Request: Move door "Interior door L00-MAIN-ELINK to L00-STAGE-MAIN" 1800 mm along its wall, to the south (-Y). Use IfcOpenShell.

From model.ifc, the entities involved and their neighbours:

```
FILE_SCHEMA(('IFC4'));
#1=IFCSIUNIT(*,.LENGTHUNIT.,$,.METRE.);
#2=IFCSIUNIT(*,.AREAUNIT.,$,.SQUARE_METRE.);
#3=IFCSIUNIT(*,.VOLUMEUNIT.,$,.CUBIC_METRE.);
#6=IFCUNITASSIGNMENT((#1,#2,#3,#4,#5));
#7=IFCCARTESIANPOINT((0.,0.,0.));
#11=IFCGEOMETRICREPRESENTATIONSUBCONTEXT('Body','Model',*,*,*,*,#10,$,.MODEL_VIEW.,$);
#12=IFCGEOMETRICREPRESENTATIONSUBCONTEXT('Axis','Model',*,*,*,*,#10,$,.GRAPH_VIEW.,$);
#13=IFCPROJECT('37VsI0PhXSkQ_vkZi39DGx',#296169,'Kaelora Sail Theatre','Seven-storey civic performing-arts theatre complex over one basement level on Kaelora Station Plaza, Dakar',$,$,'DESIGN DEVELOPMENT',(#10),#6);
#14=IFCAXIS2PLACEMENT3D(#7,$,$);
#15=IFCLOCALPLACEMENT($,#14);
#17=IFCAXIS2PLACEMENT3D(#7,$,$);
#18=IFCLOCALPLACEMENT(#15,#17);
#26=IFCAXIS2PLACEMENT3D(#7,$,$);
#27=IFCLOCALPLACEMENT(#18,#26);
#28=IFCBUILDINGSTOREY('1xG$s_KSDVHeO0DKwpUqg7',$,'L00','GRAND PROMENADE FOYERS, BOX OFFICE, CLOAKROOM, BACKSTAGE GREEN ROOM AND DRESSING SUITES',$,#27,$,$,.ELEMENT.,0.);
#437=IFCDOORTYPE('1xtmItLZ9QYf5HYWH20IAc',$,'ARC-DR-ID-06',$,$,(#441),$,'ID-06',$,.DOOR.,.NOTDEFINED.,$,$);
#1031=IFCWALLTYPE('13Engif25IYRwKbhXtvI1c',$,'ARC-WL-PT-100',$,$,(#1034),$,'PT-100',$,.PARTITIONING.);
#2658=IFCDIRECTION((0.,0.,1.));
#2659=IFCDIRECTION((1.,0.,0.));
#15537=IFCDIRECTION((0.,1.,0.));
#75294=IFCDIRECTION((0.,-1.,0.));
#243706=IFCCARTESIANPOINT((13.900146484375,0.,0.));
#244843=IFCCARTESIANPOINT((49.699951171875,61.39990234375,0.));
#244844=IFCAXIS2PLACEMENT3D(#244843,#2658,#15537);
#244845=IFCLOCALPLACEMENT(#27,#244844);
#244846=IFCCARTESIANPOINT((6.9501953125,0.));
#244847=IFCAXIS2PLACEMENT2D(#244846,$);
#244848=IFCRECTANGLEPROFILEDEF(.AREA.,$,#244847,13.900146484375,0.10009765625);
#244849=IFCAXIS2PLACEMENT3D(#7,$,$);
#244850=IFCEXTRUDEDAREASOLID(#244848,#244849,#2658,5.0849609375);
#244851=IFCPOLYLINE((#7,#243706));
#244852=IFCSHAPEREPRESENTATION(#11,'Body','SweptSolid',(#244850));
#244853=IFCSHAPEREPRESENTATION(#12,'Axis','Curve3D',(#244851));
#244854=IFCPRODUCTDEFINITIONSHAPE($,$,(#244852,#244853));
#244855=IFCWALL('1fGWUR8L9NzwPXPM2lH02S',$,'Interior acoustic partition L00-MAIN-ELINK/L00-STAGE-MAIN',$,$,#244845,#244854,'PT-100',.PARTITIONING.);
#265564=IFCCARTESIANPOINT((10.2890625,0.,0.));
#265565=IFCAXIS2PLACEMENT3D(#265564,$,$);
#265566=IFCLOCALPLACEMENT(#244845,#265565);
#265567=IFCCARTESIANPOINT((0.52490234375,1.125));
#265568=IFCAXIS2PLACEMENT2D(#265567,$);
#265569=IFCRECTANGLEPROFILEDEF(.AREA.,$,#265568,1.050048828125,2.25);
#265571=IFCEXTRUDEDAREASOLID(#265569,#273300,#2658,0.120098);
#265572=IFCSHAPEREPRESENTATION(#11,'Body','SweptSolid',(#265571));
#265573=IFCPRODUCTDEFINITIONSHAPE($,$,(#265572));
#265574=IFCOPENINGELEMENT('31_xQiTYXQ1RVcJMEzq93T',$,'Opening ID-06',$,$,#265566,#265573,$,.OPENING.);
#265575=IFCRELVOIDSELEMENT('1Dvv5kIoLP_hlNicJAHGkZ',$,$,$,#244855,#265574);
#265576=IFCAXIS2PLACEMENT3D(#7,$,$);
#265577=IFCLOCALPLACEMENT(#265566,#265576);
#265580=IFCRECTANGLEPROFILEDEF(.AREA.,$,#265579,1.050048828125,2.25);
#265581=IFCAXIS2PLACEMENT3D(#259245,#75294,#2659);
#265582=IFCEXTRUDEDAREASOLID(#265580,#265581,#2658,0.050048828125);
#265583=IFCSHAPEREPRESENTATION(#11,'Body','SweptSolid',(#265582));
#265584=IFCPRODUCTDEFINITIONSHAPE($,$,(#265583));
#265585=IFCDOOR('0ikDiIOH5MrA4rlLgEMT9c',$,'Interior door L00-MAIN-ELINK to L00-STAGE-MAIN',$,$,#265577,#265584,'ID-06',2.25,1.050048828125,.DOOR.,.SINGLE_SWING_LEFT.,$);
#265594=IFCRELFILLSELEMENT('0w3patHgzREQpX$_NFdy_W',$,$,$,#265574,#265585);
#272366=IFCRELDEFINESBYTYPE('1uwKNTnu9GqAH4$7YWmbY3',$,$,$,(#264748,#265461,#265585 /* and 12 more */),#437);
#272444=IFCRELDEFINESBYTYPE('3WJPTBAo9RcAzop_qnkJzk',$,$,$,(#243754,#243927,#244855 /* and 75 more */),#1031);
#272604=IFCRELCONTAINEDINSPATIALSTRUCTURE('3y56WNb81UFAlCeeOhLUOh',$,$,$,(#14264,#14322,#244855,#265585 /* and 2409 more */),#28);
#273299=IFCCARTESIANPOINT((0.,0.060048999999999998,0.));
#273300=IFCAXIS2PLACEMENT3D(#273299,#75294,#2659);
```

```python
import ifcopenshell
import ifcopenshell.api.geometry
import ifcopenshell.util.placement

model = ifcopenshell.open("model.ifc")

door = model.by_guid("0ikDiIOH5MrA4rlLgEMT9c")
opening = door.FillsVoids[0].RelatingOpeningElement
wall = opening.VoidsElements[0].RelatingBuildingElement

wall_matrix = ifcopenshell.util.placement.get_local_placement(wall.ObjectPlacement)
shift = wall_matrix[:3, 0] * -1.8
before = ifcopenshell.util.placement.get_local_placement(door.ObjectPlacement)[:3, 3].copy()

# The door is placed relative to its opening, so it follows when the opening moves.
matrix = ifcopenshell.util.placement.get_local_placement(opening.ObjectPlacement)
matrix[:3, 3] += shift
ifcopenshell.api.geometry.edit_object_placement(
    model, product=opening, matrix=matrix, is_si=False, should_transform_children=True
)

after = ifcopenshell.util.placement.get_local_placement(door.ObjectPlacement)[:3, 3]
print("door moved by", (after - before).round(3) + 0.0)

model.write("model_edited.ifc")
```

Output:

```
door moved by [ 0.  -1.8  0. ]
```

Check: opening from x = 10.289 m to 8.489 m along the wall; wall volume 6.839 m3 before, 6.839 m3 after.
